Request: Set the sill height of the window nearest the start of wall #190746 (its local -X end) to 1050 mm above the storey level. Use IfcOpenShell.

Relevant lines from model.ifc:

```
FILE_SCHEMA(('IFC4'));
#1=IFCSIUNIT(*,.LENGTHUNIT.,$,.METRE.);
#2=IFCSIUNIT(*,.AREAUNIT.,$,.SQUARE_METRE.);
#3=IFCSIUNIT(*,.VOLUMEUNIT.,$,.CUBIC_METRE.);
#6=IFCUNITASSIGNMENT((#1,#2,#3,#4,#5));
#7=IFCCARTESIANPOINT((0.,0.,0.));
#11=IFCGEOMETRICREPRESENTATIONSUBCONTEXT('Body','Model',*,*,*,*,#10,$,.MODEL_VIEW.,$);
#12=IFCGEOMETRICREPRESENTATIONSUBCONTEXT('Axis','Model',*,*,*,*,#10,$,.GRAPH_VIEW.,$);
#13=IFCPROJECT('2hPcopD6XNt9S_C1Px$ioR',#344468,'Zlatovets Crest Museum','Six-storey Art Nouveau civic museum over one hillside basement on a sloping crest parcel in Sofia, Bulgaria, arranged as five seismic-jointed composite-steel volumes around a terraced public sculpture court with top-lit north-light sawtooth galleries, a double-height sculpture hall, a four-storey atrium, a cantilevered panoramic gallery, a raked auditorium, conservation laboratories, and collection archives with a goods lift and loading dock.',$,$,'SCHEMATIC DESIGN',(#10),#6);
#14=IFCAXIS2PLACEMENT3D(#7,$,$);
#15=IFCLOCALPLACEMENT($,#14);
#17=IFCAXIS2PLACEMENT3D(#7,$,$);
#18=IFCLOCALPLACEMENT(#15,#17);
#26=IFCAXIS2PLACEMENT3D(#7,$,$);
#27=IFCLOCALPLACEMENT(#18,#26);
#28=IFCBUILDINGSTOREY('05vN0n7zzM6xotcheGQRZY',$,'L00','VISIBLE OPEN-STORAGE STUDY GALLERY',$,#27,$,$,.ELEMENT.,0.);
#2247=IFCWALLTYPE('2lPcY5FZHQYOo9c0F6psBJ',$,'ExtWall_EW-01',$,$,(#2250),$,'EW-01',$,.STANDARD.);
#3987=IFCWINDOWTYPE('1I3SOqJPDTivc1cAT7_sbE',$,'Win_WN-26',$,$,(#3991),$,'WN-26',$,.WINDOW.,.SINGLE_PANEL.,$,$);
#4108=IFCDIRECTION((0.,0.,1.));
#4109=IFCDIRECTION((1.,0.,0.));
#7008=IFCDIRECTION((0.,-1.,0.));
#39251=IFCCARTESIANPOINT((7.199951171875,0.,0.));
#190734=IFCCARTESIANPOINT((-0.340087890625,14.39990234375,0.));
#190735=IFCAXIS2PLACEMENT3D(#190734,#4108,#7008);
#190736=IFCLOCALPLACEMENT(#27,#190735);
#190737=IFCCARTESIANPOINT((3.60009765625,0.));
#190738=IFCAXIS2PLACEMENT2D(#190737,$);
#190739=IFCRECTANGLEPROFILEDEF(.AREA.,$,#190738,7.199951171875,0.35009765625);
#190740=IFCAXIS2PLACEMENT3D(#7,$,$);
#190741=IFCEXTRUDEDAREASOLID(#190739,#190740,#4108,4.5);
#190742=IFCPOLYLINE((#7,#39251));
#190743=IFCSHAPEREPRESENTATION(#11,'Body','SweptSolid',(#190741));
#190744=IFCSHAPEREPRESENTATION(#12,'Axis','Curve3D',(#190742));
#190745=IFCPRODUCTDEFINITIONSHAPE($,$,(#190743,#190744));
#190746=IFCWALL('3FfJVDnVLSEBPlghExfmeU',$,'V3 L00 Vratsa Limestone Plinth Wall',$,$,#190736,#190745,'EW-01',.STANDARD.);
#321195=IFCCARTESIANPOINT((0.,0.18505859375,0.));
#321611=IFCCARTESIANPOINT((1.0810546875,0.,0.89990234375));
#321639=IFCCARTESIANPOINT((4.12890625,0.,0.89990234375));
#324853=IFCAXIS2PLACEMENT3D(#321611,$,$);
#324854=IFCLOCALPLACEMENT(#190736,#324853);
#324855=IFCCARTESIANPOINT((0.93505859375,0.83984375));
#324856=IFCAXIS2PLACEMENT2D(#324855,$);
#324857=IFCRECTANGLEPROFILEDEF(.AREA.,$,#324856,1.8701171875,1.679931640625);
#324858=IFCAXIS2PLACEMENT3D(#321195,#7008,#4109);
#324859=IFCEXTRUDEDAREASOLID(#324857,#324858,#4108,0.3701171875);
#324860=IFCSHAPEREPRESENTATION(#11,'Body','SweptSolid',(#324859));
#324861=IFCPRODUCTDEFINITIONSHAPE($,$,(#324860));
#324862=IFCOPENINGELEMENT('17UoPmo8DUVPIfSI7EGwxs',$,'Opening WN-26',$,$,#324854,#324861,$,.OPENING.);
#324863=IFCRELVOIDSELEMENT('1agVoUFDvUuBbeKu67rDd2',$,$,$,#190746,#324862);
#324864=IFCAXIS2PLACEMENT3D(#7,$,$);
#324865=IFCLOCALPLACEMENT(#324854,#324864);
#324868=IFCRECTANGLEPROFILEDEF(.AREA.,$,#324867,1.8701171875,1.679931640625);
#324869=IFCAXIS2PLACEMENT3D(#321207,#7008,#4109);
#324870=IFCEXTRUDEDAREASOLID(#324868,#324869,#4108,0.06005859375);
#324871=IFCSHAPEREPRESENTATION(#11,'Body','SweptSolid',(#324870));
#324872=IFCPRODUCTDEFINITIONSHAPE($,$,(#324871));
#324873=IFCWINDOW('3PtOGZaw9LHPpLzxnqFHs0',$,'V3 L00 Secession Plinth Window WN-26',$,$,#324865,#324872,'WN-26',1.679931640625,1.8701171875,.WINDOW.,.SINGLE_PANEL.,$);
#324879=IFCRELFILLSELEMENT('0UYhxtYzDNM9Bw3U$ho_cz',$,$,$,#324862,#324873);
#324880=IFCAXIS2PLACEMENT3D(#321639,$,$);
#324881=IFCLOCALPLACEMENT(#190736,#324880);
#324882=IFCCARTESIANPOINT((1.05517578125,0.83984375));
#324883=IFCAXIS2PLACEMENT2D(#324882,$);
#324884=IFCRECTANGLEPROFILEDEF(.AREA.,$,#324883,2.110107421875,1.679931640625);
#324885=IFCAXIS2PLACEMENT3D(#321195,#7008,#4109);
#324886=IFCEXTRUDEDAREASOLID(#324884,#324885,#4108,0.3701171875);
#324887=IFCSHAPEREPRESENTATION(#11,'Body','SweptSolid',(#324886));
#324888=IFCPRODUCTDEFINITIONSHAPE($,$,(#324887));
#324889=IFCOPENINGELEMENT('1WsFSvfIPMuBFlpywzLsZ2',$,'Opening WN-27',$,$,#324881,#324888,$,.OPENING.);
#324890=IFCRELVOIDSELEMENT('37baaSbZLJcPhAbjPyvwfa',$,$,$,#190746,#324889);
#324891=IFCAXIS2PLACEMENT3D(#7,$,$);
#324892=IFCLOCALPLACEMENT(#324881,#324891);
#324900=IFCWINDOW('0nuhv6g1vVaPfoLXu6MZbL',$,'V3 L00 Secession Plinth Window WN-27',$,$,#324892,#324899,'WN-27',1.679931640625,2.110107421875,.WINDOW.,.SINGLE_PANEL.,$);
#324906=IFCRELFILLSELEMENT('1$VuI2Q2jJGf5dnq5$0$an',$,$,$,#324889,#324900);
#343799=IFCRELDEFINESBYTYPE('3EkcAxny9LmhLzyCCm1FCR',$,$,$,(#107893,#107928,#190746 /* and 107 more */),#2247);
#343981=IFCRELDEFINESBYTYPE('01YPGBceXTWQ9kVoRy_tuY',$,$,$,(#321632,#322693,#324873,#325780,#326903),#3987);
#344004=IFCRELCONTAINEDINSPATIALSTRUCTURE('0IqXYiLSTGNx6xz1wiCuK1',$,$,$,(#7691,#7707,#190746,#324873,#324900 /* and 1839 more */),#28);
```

```python
import numpy as np
import ifcopenshell
import ifcopenshell.api.geometry
import ifcopenshell.geom
import ifcopenshell.util.element
import ifcopenshell.util.placement
import ifcopenshell.util.shape
import ifcopenshell.util.unit

model = ifcopenshell.open("model.ifc")
unit_scale = ifcopenshell.util.unit.calculate_unit_scale(model)

window = model.by_guid("3PtOGZaw9LHPpLzxnqFHs0")
opening = window.FillsVoids[0].RelatingOpeningElement
storey = ifcopenshell.util.element.get_container(window, ifc_class="IfcBuildingStorey")
level = ifcopenshell.util.placement.get_local_placement(storey.ObjectPlacement)[2, 3]

# The opening's origin need not be at the sill, so measure its lowest point.
shape = ifcopenshell.geom.create_shape(ifcopenshell.geom.settings(), opening)
bottom = ifcopenshell.util.shape.get_shape_bottom_elevation(shape, shape.geometry) / unit_scale
dz = level + 1.05 - bottom

shift = np.array([0.0, 0.0, dz])
# The window is placed relative to its opening, so it follows when the opening moves.
matrix = ifcopenshell.util.placement.get_local_placement(opening.ObjectPlacement)
matrix[:3, 3] += shift
ifcopenshell.api.geometry.edit_object_placement(
    model, product=opening, matrix=matrix, is_si=False, should_transform_children=True
)

print(f"moved by {dz * unit_scale:+.3f} m")

model.write("model-out.ifc")
```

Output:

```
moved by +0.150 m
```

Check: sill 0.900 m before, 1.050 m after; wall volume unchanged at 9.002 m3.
